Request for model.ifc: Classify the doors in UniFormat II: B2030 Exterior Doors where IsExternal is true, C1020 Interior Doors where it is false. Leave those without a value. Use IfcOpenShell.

First a look at what the model holds.

```python
import ifcopenshell
import ifcopenshell.util.element

model = ifcopenshell.open("model.ifc")
print(model.schema)
print("classifications:", [c.Name for c in model.by_type("IfcClassification")])
values = [ifcopenshell.util.element.get_pset(e, "Pset_DoorCommon", "IsExternal") for e in model.by_type("IfcDoor")]
for value in (True, False, None):
    print("IsExternal", value, values.count(value))
```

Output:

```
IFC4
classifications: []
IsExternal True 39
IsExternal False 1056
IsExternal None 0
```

```python
import ifcopenshell
import ifcopenshell.api.classification
import ifcopenshell.util.element

model = ifcopenshell.open("model.ifc")

system = ifcopenshell.api.classification.add_classification(model, classification="UniFormat II")

doors = model.by_type("IfcDoor")
external = {e: ifcopenshell.util.element.get_pset(e, "Pset_DoorCommon", "IsExternal") for e in doors}
for flag, code, name in ((True, "B2030", "Exterior Doors"), (False, "C1020", "Interior Doors")):
    products = [e for e in doors if external[e] is flag]
    ifcopenshell.api.classification.add_reference(
        model, products=products, classification=system, identification=code, name=name
    )
    print(code, len(products))

model.write("model_v2.ifc")
```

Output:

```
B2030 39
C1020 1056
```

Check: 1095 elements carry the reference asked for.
